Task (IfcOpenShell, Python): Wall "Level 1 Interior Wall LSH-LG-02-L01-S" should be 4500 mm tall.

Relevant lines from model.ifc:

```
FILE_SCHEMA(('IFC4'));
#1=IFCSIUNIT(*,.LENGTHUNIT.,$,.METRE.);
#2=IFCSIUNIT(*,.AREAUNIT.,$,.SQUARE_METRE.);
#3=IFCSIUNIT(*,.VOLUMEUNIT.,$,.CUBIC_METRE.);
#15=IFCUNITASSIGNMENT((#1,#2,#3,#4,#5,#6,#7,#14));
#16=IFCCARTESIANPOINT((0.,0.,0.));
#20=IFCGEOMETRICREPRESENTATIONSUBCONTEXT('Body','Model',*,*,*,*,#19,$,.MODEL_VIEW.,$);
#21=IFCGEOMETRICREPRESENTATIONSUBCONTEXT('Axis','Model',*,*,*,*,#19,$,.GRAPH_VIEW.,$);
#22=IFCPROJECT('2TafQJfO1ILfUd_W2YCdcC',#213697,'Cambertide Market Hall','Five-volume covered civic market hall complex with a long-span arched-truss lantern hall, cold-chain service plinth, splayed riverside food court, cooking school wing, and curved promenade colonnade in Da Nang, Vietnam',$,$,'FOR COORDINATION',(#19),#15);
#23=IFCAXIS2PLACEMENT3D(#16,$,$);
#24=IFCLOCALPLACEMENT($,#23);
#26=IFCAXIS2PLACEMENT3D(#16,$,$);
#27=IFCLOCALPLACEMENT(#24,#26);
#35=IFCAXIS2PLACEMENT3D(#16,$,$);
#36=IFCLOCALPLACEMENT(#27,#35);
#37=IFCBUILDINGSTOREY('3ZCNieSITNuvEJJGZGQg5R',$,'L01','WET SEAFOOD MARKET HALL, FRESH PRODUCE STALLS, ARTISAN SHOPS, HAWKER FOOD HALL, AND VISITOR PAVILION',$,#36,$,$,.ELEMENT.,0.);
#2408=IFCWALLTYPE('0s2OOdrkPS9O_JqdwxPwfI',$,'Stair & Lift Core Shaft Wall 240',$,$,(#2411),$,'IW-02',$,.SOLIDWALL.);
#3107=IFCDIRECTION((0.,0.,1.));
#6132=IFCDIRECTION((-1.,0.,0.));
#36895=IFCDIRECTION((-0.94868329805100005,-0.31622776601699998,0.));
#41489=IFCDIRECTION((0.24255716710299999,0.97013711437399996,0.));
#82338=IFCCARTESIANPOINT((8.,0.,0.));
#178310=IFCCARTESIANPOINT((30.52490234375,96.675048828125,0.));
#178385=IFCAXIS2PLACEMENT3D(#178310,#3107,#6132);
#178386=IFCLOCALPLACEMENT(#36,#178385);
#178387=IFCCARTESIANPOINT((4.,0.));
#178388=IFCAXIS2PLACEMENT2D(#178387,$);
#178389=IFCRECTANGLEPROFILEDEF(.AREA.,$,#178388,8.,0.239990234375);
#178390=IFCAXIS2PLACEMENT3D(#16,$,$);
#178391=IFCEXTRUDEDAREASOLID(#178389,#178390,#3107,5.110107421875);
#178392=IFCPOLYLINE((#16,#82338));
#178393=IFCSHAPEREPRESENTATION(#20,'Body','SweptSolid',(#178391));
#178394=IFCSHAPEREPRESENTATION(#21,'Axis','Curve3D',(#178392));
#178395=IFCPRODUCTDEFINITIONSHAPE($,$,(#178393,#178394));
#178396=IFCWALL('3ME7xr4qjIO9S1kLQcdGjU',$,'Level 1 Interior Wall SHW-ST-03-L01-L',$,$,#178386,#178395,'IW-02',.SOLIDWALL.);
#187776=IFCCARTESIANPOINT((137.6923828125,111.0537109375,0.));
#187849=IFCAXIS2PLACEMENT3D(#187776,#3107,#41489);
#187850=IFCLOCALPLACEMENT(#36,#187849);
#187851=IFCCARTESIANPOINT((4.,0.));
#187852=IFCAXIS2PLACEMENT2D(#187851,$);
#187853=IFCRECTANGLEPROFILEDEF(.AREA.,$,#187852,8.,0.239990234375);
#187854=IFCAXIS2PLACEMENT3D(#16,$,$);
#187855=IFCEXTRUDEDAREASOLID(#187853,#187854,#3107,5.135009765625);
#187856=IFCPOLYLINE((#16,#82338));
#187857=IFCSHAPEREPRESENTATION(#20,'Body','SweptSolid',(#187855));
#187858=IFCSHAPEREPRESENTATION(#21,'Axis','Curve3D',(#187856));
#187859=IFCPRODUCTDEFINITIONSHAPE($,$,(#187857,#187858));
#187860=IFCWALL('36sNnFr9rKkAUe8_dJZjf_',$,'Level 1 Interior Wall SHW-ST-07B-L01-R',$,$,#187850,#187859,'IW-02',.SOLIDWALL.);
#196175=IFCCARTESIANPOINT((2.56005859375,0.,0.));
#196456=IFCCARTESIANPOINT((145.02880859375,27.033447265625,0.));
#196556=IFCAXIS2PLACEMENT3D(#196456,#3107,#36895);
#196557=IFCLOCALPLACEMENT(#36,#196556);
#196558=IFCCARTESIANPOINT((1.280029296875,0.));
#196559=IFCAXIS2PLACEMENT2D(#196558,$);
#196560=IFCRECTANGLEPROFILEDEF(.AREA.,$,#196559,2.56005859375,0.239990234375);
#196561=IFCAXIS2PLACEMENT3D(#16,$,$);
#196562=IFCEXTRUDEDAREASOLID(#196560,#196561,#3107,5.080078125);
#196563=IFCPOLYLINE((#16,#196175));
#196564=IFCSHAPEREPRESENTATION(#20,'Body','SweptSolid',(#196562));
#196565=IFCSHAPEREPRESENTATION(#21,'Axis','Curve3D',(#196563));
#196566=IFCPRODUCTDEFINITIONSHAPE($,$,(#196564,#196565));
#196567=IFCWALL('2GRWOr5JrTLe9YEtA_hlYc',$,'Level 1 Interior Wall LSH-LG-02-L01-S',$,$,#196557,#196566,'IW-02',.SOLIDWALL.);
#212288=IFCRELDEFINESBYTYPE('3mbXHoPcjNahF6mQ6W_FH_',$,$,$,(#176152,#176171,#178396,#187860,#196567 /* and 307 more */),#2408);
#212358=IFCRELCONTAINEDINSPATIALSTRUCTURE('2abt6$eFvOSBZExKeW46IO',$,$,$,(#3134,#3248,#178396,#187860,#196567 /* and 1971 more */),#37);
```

```python
import ifcopenshell
import ifcopenshell.geom
import ifcopenshell.util.representation
import ifcopenshell.util.shape
import ifcopenshell.util.unit

model = ifcopenshell.open("model.ifc")
unit_scale = ifcopenshell.util.unit.calculate_unit_scale(model)
settings = ifcopenshell.geom.settings()


def volume(element):
    """Net volume in cubic metres, openings subtracted."""
    shape = ifcopenshell.geom.create_shape(settings, element)
    return ifcopenshell.util.shape.get_volume(shape.geometry)


wall = model.by_id(196567)
before = volume(wall)

body = ifcopenshell.util.representation.get_representation(wall, "Model", "Body")
solid = body.Items[0]
old_height = solid.Depth
solid.Depth = 4.5 / unit_scale
after = volume(wall)

print(f"height {old_height:g} -> {solid.Depth:g}, volume {before:.3f} -> {after:.3f} m3")

model.write("model_edited.ifc")
```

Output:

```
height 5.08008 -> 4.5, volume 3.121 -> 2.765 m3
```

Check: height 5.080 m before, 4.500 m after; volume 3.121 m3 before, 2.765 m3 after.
